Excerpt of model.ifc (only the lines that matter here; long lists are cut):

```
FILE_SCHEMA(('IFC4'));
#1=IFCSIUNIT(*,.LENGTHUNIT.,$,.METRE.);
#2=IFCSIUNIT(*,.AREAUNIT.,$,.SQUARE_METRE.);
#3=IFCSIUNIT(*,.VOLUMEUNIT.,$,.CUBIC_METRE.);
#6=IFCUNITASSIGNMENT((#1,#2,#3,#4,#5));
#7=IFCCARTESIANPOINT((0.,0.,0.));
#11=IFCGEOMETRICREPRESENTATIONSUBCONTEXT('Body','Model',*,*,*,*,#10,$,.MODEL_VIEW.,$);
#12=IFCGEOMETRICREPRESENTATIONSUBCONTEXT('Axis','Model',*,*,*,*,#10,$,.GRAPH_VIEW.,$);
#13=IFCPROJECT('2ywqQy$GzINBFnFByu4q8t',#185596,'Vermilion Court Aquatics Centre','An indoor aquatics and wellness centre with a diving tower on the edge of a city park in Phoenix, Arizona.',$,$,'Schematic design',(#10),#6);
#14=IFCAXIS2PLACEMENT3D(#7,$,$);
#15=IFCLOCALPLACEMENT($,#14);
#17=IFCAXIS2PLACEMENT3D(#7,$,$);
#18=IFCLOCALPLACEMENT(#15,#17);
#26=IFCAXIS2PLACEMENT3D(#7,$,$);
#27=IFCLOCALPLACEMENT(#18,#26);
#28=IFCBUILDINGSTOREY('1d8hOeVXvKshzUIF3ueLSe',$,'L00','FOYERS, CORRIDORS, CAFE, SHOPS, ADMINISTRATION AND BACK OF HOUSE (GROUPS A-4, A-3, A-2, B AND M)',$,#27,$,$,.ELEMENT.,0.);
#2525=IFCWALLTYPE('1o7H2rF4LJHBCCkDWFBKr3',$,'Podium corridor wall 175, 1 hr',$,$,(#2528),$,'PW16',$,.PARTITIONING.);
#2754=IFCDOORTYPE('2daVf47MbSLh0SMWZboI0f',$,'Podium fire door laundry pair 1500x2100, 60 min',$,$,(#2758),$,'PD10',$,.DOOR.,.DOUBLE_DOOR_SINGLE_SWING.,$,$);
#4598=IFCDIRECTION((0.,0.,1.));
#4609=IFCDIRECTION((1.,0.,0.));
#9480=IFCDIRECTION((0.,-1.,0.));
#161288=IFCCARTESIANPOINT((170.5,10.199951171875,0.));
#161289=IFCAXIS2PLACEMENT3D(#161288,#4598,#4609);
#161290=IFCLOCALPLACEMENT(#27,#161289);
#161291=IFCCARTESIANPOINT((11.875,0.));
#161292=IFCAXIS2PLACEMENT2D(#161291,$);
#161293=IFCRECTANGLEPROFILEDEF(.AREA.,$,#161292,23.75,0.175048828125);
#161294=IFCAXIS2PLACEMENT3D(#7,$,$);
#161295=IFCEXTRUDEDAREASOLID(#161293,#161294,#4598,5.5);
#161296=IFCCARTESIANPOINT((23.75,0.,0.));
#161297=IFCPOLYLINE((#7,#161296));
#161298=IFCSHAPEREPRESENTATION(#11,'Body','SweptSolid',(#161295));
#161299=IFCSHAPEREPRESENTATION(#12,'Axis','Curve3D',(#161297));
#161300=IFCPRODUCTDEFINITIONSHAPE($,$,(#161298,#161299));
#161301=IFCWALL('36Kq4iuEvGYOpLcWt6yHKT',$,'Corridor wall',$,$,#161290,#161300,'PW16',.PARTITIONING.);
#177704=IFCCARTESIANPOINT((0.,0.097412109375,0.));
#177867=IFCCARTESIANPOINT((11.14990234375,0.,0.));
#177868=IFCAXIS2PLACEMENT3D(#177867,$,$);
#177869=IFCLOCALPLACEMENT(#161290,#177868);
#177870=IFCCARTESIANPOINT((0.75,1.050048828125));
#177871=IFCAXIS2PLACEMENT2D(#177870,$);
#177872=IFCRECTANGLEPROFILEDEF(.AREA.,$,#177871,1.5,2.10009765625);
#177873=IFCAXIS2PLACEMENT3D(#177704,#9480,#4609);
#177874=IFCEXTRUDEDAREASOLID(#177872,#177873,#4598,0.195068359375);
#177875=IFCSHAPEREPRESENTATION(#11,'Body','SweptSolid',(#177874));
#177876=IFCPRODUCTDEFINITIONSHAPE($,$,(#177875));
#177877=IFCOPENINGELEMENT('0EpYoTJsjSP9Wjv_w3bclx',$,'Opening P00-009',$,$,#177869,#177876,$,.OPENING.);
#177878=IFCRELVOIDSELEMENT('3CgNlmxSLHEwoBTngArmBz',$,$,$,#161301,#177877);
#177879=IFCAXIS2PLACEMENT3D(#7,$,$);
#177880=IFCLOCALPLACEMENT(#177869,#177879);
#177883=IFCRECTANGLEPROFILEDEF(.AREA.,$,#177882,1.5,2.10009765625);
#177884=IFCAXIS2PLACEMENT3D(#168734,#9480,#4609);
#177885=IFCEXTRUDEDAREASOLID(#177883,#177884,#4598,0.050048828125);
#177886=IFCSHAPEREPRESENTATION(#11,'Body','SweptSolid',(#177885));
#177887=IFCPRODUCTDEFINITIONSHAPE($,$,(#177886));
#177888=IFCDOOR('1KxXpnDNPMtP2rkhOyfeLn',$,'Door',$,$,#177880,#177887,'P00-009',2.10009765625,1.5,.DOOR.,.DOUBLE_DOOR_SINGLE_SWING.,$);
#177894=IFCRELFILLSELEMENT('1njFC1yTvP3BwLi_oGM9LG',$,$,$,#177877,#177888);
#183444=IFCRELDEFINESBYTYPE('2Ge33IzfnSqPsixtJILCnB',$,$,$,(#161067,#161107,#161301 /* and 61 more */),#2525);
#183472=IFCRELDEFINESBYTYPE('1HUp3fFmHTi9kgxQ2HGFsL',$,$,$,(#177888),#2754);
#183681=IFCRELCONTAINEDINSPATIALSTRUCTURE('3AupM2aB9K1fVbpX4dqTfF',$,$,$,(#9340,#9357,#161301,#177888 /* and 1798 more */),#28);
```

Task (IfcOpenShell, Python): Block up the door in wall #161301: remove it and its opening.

```python
import ifcopenshell
import ifcopenshell.api.feature
import ifcopenshell.api.root
import ifcopenshell.geom
import ifcopenshell.util.shape

model = ifcopenshell.open("model.ifc")
settings = ifcopenshell.geom.settings()


def volume(element):
    """Net volume in cubic metres, openings subtracted."""
    shape = ifcopenshell.geom.create_shape(settings, element)
    return ifcopenshell.util.shape.get_volume(shape.geometry)


door = model.by_guid("1KxXpnDNPMtP2rkhOyfeLn")
opening = door.FillsVoids[0].RelatingOpeningElement
wall = opening.VoidsElements[0].RelatingBuildingElement
before = volume(wall)

ifcopenshell.api.root.remove_product(model, product=door)
ifcopenshell.api.feature.remove_feature(model, feature=opening)

after = volume(wall)

print(f"wall volume {before:.3f} -> {after:.3f} m3")

model.write("model_updated.ifc")
```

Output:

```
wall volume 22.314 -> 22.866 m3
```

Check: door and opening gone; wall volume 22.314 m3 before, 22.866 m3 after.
